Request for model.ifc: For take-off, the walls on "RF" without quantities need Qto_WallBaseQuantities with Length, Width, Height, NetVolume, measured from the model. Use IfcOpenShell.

First a look at what the model holds.

```python
import ifcopenshell
import ifcopenshell.util.element
import ifcopenshell.util.unit

model = ifcopenshell.open("model.ifc")
print(model.schema)
for unit_type in ("LENGTHUNIT", "AREAUNIT", "VOLUMEUNIT"):
    print(unit_type, ifcopenshell.util.unit.calculate_unit_scale(model, unit_type))
storey = next(s for s in model.by_type("IfcBuildingStorey") if s.Name == "RF")
walls = [e for e in ifcopenshell.util.element.get_decomposition(storey) if e.is_a("IfcWall")]
for e in sorted(walls, key=lambda e: e.id()):
    print(e.id(), e.is_a(), e.Name, list(ifcopenshell.util.element.get_psets(e, qtos_only=True)), sep=" | ")
```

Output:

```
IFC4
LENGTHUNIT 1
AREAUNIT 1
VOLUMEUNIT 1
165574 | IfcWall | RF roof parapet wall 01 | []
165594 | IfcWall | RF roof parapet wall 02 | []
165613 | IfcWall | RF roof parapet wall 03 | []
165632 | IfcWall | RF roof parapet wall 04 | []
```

```python
import ifcopenshell
import ifcopenshell.api.pset
import ifcopenshell.geom
import ifcopenshell.util.element
import ifcopenshell.util.shape
import ifcopenshell.util.unit

model = ifcopenshell.open("model.ifc")
unit_scale = ifcopenshell.util.unit.calculate_unit_scale(model)
volume_scale = ifcopenshell.util.unit.calculate_unit_scale(model, "VOLUMEUNIT")
settings = ifcopenshell.geom.settings()

storey = next(s for s in model.by_type("IfcBuildingStorey") if s.Name == "RF")
walls = [e for e in ifcopenshell.util.element.get_decomposition(storey) if e.is_a("IfcWall")]

for e in sorted(walls, key=lambda e: e.id()):
    if ifcopenshell.util.element.get_psets(e, qtos_only=True, should_inherit=False):
        continue
    # Geometry comes back in metres, in the element's own axes.
    shape = ifcopenshell.geom.create_shape(settings, e)
    values = {
        "Length": ifcopenshell.util.shape.get_x(shape.geometry) / unit_scale,
        "Width": ifcopenshell.util.shape.get_y(shape.geometry) / unit_scale,
        "Height": ifcopenshell.util.shape.get_z(shape.geometry) / unit_scale,
        "NetVolume": ifcopenshell.util.shape.get_volume(shape.geometry) / volume_scale,
    }
    qto = ifcopenshell.api.pset.add_qto(model, product=e, name="Qto_WallBaseQuantities")
    ifcopenshell.api.pset.edit_qto(model, qto=qto, properties=values)
    print(e.id(), {k: round(v, 3) for k, v in values.items()})

model.write("model_rev.ifc")
```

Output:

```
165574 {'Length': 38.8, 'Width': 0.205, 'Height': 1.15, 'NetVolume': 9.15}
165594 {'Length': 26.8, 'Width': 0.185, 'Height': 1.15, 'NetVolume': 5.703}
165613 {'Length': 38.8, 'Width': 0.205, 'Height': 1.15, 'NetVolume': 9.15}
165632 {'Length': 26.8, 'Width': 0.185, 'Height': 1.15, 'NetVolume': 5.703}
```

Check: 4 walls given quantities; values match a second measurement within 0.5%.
